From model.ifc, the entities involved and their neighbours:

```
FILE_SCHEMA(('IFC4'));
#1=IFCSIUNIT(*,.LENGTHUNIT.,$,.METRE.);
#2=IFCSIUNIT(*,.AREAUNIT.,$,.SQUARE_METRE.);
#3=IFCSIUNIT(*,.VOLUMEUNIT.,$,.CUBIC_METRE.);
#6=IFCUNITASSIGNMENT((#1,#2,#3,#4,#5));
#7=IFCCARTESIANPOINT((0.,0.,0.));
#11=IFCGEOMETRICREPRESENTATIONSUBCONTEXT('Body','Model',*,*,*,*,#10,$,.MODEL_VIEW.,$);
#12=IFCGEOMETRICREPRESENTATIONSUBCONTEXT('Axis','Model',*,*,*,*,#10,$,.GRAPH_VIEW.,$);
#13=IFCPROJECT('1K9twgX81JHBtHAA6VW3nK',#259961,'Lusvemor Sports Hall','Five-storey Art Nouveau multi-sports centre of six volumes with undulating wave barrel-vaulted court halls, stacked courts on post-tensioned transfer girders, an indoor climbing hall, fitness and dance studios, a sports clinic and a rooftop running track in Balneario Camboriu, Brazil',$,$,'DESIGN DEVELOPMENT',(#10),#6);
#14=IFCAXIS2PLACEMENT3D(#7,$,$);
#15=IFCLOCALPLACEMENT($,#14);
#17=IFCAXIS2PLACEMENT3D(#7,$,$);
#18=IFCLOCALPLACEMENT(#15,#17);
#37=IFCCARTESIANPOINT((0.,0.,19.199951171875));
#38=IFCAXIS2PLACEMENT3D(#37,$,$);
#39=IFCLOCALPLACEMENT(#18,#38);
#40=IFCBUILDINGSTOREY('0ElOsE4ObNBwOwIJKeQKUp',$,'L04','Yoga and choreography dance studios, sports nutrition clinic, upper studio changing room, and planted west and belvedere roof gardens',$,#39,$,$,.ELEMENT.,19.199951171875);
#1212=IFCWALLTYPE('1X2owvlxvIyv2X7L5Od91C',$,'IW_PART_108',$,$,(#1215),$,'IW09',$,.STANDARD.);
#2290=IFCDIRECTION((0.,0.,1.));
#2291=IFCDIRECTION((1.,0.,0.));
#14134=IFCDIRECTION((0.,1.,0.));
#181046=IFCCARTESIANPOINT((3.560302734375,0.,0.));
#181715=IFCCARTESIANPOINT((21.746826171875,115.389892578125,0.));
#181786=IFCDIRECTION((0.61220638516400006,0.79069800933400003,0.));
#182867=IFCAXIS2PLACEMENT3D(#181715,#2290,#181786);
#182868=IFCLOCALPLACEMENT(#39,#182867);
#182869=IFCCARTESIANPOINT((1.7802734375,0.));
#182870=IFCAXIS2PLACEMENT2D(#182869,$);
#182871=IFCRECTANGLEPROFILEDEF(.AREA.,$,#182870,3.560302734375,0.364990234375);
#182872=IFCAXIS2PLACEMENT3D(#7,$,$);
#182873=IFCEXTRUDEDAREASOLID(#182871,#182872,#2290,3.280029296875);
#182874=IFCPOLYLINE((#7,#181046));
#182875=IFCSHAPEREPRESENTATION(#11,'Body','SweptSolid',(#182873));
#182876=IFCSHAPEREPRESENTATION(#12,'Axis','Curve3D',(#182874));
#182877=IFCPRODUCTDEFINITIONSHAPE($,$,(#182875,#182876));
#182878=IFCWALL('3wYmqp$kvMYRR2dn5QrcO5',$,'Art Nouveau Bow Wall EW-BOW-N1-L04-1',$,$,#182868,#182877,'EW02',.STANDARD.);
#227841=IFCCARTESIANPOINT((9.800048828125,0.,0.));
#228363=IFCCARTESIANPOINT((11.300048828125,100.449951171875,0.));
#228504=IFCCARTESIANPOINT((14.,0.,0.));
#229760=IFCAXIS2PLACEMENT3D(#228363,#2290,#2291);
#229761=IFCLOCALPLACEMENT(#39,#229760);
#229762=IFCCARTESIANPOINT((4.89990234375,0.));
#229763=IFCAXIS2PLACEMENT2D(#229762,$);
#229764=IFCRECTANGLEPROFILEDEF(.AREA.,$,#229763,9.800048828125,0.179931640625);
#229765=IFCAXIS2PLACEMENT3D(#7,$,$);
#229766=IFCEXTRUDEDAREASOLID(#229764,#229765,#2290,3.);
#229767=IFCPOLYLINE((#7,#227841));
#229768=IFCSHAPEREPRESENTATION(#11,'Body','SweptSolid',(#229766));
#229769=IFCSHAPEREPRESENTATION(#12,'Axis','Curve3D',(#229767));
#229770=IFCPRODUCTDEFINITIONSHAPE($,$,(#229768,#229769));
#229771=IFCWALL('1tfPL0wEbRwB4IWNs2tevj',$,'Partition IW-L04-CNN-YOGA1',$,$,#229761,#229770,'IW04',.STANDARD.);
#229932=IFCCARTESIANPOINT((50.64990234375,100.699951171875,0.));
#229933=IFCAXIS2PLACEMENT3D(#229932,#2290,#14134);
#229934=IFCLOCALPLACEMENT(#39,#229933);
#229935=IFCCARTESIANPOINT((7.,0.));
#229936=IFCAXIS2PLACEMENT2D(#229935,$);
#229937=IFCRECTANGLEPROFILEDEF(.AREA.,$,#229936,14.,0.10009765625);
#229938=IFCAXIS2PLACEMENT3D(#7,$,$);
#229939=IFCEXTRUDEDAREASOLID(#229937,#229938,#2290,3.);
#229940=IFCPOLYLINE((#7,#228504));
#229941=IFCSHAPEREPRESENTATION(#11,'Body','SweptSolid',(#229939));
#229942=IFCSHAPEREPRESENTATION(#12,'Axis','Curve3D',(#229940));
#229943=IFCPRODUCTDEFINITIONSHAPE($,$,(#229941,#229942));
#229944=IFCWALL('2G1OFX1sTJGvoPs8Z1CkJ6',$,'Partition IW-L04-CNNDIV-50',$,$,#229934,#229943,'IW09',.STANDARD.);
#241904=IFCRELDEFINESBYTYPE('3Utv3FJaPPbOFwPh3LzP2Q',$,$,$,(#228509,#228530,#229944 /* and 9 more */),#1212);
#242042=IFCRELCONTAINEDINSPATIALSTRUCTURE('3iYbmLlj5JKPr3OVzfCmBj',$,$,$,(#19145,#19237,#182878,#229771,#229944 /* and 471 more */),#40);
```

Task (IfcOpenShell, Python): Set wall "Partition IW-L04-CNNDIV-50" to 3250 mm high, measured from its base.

```python
import ifcopenshell
import ifcopenshell.geom
import ifcopenshell.util.representation
import ifcopenshell.util.shape

model = ifcopenshell.open("model.ifc")
settings = ifcopenshell.geom.settings()


def volume(element):
    """Net volume in cubic metres, openings subtracted."""
    shape = ifcopenshell.geom.create_shape(settings, element)
    return ifcopenshell.util.shape.get_volume(shape.geometry)


wall = model.by_guid("2G1OFX1sTJGvoPs8Z1CkJ6")
before = volume(wall)

body = ifcopenshell.util.representation.get_representation(wall, "Model", "Body")
solid = body.Items[0]
old_height = solid.Depth
solid.Depth = 3.25
after = volume(wall)

print(f"height {old_height:g} -> {solid.Depth:g}, volume {before:.3f} -> {after:.3f} m3")

model.write("model_updated.ifc")
```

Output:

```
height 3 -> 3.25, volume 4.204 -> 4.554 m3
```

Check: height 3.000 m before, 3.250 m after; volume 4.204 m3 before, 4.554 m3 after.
